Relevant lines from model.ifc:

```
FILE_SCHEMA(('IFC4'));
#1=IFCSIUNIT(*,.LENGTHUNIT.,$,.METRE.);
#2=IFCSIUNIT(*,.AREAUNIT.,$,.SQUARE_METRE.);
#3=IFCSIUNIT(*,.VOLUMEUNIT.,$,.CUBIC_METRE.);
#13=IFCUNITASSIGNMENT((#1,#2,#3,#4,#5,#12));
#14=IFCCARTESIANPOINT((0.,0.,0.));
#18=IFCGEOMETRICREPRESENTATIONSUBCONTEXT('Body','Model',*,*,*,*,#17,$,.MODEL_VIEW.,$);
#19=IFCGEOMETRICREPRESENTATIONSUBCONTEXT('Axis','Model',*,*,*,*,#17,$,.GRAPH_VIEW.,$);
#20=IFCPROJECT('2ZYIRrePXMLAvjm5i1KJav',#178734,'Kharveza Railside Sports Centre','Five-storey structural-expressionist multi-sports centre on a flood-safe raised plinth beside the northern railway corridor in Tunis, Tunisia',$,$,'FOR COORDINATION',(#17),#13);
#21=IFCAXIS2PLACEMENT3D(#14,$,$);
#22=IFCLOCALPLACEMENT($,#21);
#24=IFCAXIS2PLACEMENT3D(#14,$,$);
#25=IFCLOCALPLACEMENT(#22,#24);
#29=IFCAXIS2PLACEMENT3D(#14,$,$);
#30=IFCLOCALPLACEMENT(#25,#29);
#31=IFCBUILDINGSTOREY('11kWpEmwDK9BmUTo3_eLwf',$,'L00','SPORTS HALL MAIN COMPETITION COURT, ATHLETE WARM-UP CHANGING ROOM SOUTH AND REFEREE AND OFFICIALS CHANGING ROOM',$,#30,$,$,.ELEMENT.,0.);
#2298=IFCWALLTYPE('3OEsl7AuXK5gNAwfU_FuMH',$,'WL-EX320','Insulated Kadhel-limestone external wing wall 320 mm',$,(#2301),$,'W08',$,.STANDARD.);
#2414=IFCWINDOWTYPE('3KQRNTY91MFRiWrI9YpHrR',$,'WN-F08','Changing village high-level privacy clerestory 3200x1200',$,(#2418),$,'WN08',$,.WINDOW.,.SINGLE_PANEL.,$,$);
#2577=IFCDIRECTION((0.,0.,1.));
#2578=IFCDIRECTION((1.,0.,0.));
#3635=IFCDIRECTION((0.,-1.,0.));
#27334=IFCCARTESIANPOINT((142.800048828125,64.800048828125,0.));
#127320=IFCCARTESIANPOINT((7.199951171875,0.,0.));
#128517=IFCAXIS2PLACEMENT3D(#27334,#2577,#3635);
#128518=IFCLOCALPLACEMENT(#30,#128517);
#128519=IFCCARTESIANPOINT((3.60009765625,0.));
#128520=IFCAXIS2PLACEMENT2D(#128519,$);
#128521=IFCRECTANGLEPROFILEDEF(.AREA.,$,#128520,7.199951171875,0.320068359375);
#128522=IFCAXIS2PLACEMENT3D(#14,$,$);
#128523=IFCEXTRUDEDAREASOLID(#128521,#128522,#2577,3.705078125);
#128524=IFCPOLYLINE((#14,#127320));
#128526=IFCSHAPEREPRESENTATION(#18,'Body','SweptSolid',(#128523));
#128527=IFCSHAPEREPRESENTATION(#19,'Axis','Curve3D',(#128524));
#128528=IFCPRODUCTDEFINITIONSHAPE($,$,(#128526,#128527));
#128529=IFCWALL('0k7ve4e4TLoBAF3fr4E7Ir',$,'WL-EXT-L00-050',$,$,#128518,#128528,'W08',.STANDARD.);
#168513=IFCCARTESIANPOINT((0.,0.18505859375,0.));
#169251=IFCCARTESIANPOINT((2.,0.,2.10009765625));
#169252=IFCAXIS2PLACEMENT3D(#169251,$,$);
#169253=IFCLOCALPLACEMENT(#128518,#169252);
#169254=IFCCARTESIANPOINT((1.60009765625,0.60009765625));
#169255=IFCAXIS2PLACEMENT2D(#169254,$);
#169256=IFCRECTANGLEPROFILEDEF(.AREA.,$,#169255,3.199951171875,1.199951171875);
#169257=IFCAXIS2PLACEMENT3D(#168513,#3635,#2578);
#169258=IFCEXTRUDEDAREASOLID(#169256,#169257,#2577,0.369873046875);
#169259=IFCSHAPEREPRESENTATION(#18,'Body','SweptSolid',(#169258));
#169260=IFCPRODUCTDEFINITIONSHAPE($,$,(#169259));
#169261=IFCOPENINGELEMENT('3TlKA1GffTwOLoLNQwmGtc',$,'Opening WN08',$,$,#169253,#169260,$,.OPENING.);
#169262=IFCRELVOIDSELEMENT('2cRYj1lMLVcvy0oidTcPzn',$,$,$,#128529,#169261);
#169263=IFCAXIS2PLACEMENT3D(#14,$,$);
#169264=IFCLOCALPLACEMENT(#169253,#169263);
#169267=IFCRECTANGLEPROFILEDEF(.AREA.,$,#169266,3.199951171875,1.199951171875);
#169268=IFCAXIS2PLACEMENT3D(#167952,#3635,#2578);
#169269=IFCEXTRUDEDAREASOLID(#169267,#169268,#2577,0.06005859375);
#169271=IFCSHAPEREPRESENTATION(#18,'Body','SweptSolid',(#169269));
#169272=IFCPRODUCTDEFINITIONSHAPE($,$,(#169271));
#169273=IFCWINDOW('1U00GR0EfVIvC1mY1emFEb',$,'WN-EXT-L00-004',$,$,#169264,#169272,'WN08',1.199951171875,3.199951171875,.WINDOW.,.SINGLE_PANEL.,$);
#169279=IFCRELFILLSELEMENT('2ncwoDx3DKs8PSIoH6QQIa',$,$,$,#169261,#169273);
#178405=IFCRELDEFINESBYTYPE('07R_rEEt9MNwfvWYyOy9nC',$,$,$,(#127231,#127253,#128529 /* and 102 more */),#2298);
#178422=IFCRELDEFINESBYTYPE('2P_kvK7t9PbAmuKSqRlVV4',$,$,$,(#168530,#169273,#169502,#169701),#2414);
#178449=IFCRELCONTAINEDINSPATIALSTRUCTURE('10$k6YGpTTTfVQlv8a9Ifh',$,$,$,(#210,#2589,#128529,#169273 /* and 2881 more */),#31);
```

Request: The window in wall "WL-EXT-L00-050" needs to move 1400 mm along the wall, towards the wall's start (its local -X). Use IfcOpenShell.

```python
import ifcopenshell
import ifcopenshell.api.geometry
import ifcopenshell.util.placement
import ifcopenshell.util.unit

model = ifcopenshell.open("model.ifc")
unit_scale = ifcopenshell.util.unit.calculate_unit_scale(model)

window = model.by_guid("1U00GR0EfVIvC1mY1emFEb")
opening = window.FillsVoids[0].RelatingOpeningElement
wall = opening.VoidsElements[0].RelatingBuildingElement

wall_matrix = ifcopenshell.util.placement.get_local_placement(wall.ObjectPlacement)
shift = wall_matrix[:3, 0] * -1.4 / unit_scale
before = ifcopenshell.util.placement.get_local_placement(window.ObjectPlacement)[:3, 3].copy()

# The window is placed relative to its opening, so it follows when the opening moves.
matrix = ifcopenshell.util.placement.get_local_placement(opening.ObjectPlacement)
matrix[:3, 3] += shift
ifcopenshell.api.geometry.edit_object_placement(
    model, product=opening, matrix=matrix, is_si=False, should_transform_children=True
)

after = ifcopenshell.util.placement.get_local_placement(window.ObjectPlacement)[:3, 3]
print("window moved by", (after - before).round(3) + 0.0)

model.write("model_v2.ifc")
```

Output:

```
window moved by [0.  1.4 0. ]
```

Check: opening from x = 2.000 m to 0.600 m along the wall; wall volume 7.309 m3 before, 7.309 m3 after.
